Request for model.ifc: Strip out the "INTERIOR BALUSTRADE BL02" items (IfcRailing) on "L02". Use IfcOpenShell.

First a look at what the model holds.

```python
import ifcopenshell
import ifcopenshell.util.element

model = ifcopenshell.open("model.ifc")
print(model.schema)
storey = next(s for s in model.by_type("IfcBuildingStorey") if s.Name == "L02")
railings = [e for e in ifcopenshell.util.element.get_decomposition(storey) if e.is_a("IfcRailing")]
seen = {}
for e in railings:
    element_type = ifcopenshell.util.element.get_type(e)
    name = element_type.Name if element_type not in (None, e) else None
    seen[name] = seen.get(name, 0) + 1
for name, count in sorted(seen.items(), key=str):
    print(count, "x", name)
```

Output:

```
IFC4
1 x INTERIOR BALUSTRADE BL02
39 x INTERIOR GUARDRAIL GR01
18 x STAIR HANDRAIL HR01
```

```python
import ifcopenshell
import ifcopenshell.api.root
import ifcopenshell.util.element

model = ifcopenshell.open("model.ifc")

storey = next(s for s in model.by_type("IfcBuildingStorey") if s.Name == "L02")
railings = [e for e in ifcopenshell.util.element.get_decomposition(storey) if e.is_a("IfcRailing")]
targets = [e for e in railings if (t := ifcopenshell.util.element.get_type(e)) not in (None, e) and t.Name == "INTERIOR BALUSTRADE BL02"]

for e in targets:
    ifcopenshell.api.root.remove_product(model, product=e)
print(len(targets), "removed")

model.write("model_v2.ifc")
```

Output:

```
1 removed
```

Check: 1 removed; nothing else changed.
